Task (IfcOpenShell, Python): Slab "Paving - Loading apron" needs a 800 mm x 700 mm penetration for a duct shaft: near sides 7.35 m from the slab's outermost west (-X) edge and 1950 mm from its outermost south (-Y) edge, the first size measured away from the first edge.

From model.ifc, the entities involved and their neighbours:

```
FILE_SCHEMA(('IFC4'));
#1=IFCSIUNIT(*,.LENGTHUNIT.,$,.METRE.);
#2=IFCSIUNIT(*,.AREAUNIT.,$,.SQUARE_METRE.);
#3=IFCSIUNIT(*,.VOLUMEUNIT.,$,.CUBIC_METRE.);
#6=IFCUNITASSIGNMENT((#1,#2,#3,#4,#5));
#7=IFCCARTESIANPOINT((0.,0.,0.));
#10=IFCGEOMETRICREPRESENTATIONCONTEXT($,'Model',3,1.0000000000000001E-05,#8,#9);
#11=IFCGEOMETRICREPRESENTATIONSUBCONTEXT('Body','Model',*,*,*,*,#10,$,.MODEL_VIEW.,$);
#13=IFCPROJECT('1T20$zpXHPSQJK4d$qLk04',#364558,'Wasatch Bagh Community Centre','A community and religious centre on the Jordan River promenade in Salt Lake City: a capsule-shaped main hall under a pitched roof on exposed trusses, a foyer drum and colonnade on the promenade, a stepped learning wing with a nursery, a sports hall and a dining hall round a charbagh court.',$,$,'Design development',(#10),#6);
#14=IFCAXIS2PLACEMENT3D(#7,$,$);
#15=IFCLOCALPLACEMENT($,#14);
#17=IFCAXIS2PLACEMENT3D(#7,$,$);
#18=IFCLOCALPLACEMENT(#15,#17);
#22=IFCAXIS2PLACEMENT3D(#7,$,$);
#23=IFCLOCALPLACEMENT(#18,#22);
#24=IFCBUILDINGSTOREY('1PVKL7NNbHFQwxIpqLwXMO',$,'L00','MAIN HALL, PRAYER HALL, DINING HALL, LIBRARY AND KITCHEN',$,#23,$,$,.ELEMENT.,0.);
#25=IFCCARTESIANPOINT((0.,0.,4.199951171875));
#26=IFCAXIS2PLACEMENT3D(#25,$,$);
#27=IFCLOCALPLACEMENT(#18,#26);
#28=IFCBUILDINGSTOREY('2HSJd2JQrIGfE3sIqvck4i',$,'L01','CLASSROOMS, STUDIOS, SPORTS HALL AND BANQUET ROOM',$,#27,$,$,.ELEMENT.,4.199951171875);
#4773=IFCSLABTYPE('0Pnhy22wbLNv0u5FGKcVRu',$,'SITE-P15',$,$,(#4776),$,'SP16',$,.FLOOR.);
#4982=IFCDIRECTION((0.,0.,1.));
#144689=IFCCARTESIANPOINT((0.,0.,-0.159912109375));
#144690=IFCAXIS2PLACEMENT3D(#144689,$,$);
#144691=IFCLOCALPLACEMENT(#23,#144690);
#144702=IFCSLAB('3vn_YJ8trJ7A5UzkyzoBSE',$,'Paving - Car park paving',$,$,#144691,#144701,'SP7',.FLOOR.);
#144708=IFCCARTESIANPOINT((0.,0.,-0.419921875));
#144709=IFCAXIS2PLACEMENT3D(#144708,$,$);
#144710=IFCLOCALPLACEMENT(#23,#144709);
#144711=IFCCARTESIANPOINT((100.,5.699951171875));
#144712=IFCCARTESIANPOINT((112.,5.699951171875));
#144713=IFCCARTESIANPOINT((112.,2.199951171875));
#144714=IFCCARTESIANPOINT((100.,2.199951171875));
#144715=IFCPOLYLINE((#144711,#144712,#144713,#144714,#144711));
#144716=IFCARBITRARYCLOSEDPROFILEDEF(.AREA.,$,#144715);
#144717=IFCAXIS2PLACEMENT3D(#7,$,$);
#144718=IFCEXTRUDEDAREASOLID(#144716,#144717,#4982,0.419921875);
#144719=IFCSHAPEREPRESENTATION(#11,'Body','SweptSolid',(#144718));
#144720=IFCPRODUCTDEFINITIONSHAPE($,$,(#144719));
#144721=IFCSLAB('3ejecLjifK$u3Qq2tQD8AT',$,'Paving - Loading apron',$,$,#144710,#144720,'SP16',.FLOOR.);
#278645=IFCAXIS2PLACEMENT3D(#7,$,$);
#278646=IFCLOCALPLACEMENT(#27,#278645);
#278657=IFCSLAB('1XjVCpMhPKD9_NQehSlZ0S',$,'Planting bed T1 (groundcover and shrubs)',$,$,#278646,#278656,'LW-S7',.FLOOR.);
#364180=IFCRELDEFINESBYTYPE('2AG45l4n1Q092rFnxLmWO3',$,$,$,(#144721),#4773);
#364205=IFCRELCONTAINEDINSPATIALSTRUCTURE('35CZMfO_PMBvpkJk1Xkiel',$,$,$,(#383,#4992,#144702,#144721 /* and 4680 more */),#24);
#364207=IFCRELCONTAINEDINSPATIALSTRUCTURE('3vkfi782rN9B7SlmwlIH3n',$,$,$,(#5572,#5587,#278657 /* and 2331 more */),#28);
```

```python
import numpy as np
import ifcopenshell
import ifcopenshell.api.feature
import ifcopenshell.api.geometry
import ifcopenshell.api.root
import ifcopenshell.geom
import ifcopenshell.util.placement
import ifcopenshell.util.representation
import ifcopenshell.util.shape
import ifcopenshell.util.unit

model = ifcopenshell.open("model.ifc")
unit_scale = ifcopenshell.util.unit.calculate_unit_scale(model)
settings = ifcopenshell.geom.settings()


def volume(element):
    """Net volume in cubic metres, openings subtracted."""
    shape = ifcopenshell.geom.create_shape(settings, element)
    return ifcopenshell.util.shape.get_volume(shape.geometry)


slab = model.by_guid("3ejecLjifK$u3Qq2tQD8AT")
before = volume(slab)

# Extent in the slab's own axes, in metres. The edges named are its -X and -Y sides.
slab_shape = ifcopenshell.geom.create_shape(settings, slab)
vertices = ifcopenshell.util.shape.get_vertices(slab_shape.geometry)
x_min, y_min, bottom = vertices.min(axis=0)
top = vertices[:, 2].max()

opening = ifcopenshell.api.root.create_entity(model, ifc_class="IfcOpeningElement", name="Duct shaft opening", predefined_type="OPENING")
context = ifcopenshell.util.representation.get_context(model, "Model", "Body", "MODEL_VIEW")
width, depth = 0.8, 0.7
outline = [(0.0, 0.0), (width, 0.0), (width, depth), (0.0, depth), (0.0, 0.0)]
# Overshoot both faces by 50 mm so the cut is clean.
shape = ifcopenshell.api.geometry.add_slab_representation(
    model, context=context, depth=top - bottom + 0.1, polyline=outline
)
ifcopenshell.api.geometry.assign_representation(model, product=opening, representation=shape)

matrix = ifcopenshell.util.placement.get_local_placement(slab.ObjectPlacement)
matrix[:, 3] = matrix @ np.append(np.array([x_min + 7.35, y_min + 1.95, bottom - 0.05]) / unit_scale, 1.0)
ifcopenshell.api.geometry.edit_object_placement(model, product=opening, matrix=matrix, is_si=False)
ifcopenshell.api.feature.add_feature(model, feature=opening, element=slab)

after = volume(slab)

print(f"slab volume {before:.3f} -> {after:.3f} m3")

model.write("model_rev.ifc")
```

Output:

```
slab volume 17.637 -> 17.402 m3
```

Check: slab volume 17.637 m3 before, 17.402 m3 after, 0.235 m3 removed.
